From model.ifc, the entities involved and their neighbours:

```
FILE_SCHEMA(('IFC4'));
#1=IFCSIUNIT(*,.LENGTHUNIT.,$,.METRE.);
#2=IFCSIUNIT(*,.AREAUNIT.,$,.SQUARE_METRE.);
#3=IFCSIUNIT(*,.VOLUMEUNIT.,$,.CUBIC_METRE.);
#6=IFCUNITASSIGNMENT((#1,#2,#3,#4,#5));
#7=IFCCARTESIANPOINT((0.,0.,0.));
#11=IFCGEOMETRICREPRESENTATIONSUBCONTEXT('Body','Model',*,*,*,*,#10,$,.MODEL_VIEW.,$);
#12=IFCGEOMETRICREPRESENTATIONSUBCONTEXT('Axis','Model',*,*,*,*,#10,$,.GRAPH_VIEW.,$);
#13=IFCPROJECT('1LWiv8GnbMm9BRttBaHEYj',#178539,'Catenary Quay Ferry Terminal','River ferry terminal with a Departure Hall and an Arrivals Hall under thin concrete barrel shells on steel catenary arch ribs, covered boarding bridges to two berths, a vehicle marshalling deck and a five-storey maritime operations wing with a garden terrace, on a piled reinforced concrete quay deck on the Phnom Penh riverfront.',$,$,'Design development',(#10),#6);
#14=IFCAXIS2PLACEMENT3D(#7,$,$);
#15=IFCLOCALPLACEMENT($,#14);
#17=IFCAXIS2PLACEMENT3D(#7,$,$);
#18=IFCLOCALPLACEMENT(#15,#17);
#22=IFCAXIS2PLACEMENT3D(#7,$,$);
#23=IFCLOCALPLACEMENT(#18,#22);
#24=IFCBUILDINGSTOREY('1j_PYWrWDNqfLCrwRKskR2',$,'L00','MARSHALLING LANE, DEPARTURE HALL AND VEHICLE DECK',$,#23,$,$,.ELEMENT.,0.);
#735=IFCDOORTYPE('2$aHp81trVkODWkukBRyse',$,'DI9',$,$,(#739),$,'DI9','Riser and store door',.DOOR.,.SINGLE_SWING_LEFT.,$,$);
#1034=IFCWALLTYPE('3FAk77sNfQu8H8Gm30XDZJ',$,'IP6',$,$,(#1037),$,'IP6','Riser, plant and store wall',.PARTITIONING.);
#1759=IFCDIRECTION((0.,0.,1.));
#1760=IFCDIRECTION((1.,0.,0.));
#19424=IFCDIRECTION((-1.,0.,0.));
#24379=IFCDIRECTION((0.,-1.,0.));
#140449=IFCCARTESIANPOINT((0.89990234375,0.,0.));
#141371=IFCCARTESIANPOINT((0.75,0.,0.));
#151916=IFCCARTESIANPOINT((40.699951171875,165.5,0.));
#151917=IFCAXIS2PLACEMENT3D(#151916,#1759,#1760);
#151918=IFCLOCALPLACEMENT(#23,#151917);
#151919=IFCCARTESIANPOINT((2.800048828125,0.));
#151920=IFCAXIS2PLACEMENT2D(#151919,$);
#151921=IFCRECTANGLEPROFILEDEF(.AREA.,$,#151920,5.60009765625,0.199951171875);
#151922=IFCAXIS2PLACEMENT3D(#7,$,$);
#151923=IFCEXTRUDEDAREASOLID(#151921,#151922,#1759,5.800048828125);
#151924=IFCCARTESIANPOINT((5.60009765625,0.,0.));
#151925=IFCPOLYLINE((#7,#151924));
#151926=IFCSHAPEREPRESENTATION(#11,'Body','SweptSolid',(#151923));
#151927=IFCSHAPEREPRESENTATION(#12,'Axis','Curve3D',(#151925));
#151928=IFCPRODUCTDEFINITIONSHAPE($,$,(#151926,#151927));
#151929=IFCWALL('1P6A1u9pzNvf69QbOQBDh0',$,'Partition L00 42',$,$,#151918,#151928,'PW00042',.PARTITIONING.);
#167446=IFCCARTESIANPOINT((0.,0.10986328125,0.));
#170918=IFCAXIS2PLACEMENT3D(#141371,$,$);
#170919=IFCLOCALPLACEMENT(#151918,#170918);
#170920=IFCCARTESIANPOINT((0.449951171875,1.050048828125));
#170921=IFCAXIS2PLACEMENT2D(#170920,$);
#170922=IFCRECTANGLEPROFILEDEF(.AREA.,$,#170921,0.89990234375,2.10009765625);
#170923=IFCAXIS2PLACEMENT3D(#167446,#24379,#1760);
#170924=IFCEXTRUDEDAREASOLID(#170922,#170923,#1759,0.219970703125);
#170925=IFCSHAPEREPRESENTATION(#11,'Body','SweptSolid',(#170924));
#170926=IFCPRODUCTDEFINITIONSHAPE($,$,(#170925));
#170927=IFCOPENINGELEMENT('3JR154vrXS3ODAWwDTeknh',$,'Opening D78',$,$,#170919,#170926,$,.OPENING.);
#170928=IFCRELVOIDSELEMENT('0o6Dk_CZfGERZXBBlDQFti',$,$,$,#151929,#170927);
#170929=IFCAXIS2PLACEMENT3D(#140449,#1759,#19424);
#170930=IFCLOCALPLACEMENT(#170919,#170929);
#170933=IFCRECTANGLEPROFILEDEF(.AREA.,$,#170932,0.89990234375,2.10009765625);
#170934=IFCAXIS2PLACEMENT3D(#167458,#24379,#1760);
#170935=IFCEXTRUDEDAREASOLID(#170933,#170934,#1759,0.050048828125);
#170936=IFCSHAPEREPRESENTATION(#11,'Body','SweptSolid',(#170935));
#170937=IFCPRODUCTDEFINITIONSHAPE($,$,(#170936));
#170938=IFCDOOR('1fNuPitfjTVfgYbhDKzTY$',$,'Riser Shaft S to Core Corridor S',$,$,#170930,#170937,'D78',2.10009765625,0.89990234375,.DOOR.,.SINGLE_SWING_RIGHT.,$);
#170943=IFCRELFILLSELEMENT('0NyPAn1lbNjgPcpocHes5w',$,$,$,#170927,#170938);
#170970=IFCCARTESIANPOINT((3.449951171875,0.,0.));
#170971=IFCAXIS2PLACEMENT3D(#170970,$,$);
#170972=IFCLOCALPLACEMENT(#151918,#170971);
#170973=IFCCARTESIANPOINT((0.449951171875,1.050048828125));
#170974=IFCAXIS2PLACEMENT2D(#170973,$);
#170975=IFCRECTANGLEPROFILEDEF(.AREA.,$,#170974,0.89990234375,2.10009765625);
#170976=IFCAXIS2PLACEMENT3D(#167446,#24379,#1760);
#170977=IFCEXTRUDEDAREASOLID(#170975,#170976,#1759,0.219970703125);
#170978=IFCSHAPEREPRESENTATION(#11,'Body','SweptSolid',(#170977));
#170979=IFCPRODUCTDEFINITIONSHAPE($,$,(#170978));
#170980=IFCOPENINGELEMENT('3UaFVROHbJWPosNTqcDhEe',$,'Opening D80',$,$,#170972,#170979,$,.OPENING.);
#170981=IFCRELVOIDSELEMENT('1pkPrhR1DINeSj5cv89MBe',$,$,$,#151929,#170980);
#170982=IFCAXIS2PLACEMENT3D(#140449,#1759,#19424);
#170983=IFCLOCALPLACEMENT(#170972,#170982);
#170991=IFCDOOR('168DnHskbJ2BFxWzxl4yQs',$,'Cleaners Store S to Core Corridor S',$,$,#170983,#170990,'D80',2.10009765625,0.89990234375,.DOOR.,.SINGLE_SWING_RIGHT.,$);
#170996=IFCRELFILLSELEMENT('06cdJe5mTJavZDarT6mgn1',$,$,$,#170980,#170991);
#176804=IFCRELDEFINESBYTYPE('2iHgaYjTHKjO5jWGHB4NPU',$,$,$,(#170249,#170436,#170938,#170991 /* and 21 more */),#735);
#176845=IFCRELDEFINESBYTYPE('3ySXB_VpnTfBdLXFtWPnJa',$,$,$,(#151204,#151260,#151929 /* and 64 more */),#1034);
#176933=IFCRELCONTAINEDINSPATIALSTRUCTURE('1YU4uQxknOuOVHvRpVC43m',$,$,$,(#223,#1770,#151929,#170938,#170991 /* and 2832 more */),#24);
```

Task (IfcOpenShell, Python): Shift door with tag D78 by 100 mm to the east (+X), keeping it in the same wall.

```python
import ifcopenshell
import ifcopenshell.api.geometry
import ifcopenshell.util.placement

model = ifcopenshell.open("model.ifc")

door = model.by_guid("1fNuPitfjTVfgYbhDKzTY$")
opening = door.FillsVoids[0].RelatingOpeningElement
wall = opening.VoidsElements[0].RelatingBuildingElement

wall_matrix = ifcopenshell.util.placement.get_local_placement(wall.ObjectPlacement)
shift = wall_matrix[:3, 0] * 0.1
before = ifcopenshell.util.placement.get_local_placement(door.ObjectPlacement)[:3, 3].copy()

# The door is placed relative to its opening, so it follows when the opening moves.
matrix = ifcopenshell.util.placement.get_local_placement(opening.ObjectPlacement)
matrix[:3, 3] += shift
ifcopenshell.api.geometry.edit_object_placement(
    model, product=opening, matrix=matrix, is_si=False, should_transform_children=True
)

after = ifcopenshell.util.placement.get_local_placement(door.ObjectPlacement)[:3, 3]
print("door moved by", (after - before).round(3) + 0.0)

model.write("model_updated.ifc")
```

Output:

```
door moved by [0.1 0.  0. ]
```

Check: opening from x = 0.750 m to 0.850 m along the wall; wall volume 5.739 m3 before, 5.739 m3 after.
